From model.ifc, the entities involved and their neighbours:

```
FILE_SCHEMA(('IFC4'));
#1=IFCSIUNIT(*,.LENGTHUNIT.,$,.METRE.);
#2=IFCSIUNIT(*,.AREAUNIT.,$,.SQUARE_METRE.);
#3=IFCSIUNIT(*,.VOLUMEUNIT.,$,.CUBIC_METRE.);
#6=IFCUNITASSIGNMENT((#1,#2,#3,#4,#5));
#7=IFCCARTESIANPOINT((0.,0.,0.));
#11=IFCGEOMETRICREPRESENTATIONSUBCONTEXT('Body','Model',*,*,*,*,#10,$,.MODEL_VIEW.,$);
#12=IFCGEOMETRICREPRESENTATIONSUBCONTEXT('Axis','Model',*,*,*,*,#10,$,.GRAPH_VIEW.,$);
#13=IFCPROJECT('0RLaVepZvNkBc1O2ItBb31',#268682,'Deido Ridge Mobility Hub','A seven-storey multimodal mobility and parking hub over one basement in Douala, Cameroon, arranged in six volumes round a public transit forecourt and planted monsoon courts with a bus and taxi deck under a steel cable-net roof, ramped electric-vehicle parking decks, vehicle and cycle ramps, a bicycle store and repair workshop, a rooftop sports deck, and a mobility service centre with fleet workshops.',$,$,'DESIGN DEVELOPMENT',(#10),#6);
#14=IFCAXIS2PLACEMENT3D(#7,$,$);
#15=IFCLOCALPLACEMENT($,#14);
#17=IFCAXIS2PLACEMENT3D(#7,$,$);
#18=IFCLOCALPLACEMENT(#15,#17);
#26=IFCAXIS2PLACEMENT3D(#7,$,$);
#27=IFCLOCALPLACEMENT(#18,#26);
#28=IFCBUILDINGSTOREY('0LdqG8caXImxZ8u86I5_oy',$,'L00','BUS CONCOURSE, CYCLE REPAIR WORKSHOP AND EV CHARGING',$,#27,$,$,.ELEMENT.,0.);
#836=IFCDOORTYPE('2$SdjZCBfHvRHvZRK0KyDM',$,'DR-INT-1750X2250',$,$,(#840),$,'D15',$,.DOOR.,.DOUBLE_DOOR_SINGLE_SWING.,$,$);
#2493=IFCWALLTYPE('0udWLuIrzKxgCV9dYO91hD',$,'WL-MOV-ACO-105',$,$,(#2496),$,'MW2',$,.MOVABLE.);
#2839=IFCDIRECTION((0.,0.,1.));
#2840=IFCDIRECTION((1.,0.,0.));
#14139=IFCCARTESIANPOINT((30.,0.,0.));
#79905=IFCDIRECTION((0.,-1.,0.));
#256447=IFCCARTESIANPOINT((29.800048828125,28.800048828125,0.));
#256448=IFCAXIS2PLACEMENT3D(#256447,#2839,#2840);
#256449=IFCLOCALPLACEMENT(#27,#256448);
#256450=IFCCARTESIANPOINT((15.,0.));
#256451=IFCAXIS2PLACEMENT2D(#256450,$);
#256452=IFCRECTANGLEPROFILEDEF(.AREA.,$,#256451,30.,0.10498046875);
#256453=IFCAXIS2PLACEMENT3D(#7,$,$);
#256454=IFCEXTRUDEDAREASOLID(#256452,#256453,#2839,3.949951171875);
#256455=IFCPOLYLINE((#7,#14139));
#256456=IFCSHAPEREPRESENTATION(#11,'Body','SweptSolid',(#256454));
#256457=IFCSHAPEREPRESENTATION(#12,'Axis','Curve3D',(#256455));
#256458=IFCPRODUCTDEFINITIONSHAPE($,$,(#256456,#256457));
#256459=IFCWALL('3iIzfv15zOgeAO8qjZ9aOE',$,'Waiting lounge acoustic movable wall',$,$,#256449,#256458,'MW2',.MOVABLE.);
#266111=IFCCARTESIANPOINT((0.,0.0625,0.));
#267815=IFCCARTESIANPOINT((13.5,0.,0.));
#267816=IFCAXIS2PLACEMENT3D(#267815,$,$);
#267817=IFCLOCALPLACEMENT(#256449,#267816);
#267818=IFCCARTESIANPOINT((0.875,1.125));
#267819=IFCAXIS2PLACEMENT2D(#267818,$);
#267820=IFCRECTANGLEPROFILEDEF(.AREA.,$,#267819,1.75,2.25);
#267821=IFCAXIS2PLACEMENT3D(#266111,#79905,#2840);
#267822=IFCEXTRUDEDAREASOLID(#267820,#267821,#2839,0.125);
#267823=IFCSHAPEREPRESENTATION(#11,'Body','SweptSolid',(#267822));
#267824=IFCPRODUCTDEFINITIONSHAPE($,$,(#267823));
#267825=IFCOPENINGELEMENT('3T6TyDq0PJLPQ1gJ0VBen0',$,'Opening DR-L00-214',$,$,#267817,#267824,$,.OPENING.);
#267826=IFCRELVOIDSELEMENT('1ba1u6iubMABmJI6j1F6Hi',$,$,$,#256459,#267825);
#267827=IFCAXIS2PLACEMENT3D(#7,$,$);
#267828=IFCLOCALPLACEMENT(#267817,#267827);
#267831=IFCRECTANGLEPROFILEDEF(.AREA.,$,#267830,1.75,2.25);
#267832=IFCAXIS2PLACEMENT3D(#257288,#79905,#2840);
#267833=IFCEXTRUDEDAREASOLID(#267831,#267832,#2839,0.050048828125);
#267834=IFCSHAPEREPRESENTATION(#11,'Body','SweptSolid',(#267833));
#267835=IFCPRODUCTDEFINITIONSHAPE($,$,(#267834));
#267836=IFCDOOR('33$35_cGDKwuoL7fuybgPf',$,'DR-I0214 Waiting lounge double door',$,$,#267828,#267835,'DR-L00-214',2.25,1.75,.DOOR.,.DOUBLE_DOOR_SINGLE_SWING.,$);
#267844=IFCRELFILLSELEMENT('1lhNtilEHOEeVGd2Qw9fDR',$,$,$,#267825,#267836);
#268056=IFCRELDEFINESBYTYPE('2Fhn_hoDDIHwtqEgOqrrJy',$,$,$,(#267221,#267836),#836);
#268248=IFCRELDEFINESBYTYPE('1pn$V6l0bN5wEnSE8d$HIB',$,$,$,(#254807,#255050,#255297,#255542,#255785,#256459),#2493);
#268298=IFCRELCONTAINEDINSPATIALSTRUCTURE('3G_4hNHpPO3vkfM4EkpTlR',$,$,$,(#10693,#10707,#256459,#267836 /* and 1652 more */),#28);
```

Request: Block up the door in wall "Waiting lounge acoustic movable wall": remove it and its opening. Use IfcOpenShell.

```python
import ifcopenshell
import ifcopenshell.api.feature
import ifcopenshell.api.root
import ifcopenshell.geom
import ifcopenshell.util.shape

model = ifcopenshell.open("model.ifc")
settings = ifcopenshell.geom.settings()


def volume(element):
    """Net volume in cubic metres, openings subtracted."""
    shape = ifcopenshell.geom.create_shape(settings, element)
    return ifcopenshell.util.shape.get_volume(shape.geometry)


door = model.by_guid("33$35_cGDKwuoL7fuybgPf")
opening = door.FillsVoids[0].RelatingOpeningElement
wall = opening.VoidsElements[0].RelatingBuildingElement
before = volume(wall)

ifcopenshell.api.root.remove_product(model, product=door)
ifcopenshell.api.feature.remove_feature(model, feature=opening)

after = volume(wall)

print(f"wall volume {before:.3f} -> {after:.3f} m3")

model.write("model-out.ifc")
```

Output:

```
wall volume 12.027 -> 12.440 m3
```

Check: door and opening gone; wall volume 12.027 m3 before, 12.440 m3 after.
